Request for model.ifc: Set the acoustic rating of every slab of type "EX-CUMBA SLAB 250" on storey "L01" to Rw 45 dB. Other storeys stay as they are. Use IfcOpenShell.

First a look at what the model holds.

```python
import ifcopenshell
import ifcopenshell.util.element

model = ifcopenshell.open("model.ifc")
print(model.schema)
storey = next(s for s in model.by_type("IfcBuildingStorey") if s.Name == "L01")
slabs = [e for e in ifcopenshell.util.element.get_decomposition(storey) if e.is_a("IfcSlab")]
seen = {}
for e in slabs:
    element_type = ifcopenshell.util.element.get_type(e)
    key = (element_type.Name if element_type != e and element_type else None, ifcopenshell.util.element.get_pset(e, "Pset_SlabCommon", "AcousticRating"))
    seen[key] = seen.get(key, 0) + 1
for (name, value), count in sorted(seen.items(), key=str):
    print(count, "x", name, "|", value)
```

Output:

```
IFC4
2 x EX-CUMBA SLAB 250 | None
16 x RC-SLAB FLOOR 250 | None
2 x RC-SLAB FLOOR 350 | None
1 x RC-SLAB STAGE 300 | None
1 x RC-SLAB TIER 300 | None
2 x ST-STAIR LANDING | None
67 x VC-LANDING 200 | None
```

```python
import ifcopenshell
import ifcopenshell.api.pset
import ifcopenshell.util.element

model = ifcopenshell.open("model.ifc")

storey = next(s for s in model.by_type("IfcBuildingStorey") if s.Name == "L01")
slabs = [e for e in ifcopenshell.util.element.get_decomposition(storey) if e.is_a("IfcSlab")]

count = 0
for e in slabs:
    element_type = ifcopenshell.util.element.get_type(e)
    if element_type in (None, e) or element_type.Name != "EX-CUMBA SLAB 250":
        continue
    # add_pset returns the element's existing set when there is one.
    pset = ifcopenshell.api.pset.add_pset(model, product=e, name="Pset_SlabCommon")
    ifcopenshell.api.pset.edit_pset(model, pset=pset, properties={"AcousticRating": "Rw 45 dB"})
    count += 1

print(count, "slabs updated")

model.write("model_v2.ifc")
```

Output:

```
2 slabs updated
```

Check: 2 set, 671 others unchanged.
